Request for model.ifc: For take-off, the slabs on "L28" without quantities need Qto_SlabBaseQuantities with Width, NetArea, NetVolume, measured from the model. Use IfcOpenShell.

First a look at what the model holds.

```python
import ifcopenshell
import ifcopenshell.util.element
import ifcopenshell.util.unit

model = ifcopenshell.open("model.ifc")
print(model.schema)
for unit_type in ("LENGTHUNIT", "AREAUNIT", "VOLUMEUNIT"):
    print(unit_type, ifcopenshell.util.unit.calculate_unit_scale(model, unit_type))
storey = next(s for s in model.by_type("IfcBuildingStorey") if s.Name == "L28")
slabs = [e for e in ifcopenshell.util.element.get_decomposition(storey) if e.is_a("IfcSlab")]
for e in sorted(slabs, key=lambda e: e.id()):
    print(e.id(), e.is_a(), e.Name, list(ifcopenshell.util.element.get_psets(e, qtos_only=True)), sep=" | ")
```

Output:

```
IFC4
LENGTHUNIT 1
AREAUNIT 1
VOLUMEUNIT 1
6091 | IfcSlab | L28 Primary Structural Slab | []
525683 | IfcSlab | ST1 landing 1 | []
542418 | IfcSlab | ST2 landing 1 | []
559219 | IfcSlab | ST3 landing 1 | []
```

```python
import ifcopenshell
import ifcopenshell.api.pset
import ifcopenshell.geom
import ifcopenshell.util.element
import ifcopenshell.util.shape
import ifcopenshell.util.unit

model = ifcopenshell.open("model.ifc")
unit_scale = ifcopenshell.util.unit.calculate_unit_scale(model)
area_scale = ifcopenshell.util.unit.calculate_unit_scale(model, "AREAUNIT")
volume_scale = ifcopenshell.util.unit.calculate_unit_scale(model, "VOLUMEUNIT")
settings = ifcopenshell.geom.settings()

storey = next(s for s in model.by_type("IfcBuildingStorey") if s.Name == "L28")
slabs = [e for e in ifcopenshell.util.element.get_decomposition(storey) if e.is_a("IfcSlab")]

for e in sorted(slabs, key=lambda e: e.id()):
    if ifcopenshell.util.element.get_psets(e, qtos_only=True, should_inherit=False):
        continue
    # Geometry comes back in metres, in the element's own axes.
    shape = ifcopenshell.geom.create_shape(settings, e)
    values = {
        "Width": ifcopenshell.util.shape.get_z(shape.geometry) / unit_scale,
        "NetArea": ifcopenshell.util.shape.get_footprint_area(shape.geometry) / area_scale,
        "NetVolume": ifcopenshell.util.shape.get_volume(shape.geometry) / volume_scale,
    }
    qto = ifcopenshell.api.pset.add_qto(model, product=e, name="Qto_SlabBaseQuantities")
    ifcopenshell.api.pset.edit_qto(model, qto=qto, properties=values)
    print(e.id(), {k: round(v, 3) for k, v in values.items()})

model.write("model_v2.ifc")
```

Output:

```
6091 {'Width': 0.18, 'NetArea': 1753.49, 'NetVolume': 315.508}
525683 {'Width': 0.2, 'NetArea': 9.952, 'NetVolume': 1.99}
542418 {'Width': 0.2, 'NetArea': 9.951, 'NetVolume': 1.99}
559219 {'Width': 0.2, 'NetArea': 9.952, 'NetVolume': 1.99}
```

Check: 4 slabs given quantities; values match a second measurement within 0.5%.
